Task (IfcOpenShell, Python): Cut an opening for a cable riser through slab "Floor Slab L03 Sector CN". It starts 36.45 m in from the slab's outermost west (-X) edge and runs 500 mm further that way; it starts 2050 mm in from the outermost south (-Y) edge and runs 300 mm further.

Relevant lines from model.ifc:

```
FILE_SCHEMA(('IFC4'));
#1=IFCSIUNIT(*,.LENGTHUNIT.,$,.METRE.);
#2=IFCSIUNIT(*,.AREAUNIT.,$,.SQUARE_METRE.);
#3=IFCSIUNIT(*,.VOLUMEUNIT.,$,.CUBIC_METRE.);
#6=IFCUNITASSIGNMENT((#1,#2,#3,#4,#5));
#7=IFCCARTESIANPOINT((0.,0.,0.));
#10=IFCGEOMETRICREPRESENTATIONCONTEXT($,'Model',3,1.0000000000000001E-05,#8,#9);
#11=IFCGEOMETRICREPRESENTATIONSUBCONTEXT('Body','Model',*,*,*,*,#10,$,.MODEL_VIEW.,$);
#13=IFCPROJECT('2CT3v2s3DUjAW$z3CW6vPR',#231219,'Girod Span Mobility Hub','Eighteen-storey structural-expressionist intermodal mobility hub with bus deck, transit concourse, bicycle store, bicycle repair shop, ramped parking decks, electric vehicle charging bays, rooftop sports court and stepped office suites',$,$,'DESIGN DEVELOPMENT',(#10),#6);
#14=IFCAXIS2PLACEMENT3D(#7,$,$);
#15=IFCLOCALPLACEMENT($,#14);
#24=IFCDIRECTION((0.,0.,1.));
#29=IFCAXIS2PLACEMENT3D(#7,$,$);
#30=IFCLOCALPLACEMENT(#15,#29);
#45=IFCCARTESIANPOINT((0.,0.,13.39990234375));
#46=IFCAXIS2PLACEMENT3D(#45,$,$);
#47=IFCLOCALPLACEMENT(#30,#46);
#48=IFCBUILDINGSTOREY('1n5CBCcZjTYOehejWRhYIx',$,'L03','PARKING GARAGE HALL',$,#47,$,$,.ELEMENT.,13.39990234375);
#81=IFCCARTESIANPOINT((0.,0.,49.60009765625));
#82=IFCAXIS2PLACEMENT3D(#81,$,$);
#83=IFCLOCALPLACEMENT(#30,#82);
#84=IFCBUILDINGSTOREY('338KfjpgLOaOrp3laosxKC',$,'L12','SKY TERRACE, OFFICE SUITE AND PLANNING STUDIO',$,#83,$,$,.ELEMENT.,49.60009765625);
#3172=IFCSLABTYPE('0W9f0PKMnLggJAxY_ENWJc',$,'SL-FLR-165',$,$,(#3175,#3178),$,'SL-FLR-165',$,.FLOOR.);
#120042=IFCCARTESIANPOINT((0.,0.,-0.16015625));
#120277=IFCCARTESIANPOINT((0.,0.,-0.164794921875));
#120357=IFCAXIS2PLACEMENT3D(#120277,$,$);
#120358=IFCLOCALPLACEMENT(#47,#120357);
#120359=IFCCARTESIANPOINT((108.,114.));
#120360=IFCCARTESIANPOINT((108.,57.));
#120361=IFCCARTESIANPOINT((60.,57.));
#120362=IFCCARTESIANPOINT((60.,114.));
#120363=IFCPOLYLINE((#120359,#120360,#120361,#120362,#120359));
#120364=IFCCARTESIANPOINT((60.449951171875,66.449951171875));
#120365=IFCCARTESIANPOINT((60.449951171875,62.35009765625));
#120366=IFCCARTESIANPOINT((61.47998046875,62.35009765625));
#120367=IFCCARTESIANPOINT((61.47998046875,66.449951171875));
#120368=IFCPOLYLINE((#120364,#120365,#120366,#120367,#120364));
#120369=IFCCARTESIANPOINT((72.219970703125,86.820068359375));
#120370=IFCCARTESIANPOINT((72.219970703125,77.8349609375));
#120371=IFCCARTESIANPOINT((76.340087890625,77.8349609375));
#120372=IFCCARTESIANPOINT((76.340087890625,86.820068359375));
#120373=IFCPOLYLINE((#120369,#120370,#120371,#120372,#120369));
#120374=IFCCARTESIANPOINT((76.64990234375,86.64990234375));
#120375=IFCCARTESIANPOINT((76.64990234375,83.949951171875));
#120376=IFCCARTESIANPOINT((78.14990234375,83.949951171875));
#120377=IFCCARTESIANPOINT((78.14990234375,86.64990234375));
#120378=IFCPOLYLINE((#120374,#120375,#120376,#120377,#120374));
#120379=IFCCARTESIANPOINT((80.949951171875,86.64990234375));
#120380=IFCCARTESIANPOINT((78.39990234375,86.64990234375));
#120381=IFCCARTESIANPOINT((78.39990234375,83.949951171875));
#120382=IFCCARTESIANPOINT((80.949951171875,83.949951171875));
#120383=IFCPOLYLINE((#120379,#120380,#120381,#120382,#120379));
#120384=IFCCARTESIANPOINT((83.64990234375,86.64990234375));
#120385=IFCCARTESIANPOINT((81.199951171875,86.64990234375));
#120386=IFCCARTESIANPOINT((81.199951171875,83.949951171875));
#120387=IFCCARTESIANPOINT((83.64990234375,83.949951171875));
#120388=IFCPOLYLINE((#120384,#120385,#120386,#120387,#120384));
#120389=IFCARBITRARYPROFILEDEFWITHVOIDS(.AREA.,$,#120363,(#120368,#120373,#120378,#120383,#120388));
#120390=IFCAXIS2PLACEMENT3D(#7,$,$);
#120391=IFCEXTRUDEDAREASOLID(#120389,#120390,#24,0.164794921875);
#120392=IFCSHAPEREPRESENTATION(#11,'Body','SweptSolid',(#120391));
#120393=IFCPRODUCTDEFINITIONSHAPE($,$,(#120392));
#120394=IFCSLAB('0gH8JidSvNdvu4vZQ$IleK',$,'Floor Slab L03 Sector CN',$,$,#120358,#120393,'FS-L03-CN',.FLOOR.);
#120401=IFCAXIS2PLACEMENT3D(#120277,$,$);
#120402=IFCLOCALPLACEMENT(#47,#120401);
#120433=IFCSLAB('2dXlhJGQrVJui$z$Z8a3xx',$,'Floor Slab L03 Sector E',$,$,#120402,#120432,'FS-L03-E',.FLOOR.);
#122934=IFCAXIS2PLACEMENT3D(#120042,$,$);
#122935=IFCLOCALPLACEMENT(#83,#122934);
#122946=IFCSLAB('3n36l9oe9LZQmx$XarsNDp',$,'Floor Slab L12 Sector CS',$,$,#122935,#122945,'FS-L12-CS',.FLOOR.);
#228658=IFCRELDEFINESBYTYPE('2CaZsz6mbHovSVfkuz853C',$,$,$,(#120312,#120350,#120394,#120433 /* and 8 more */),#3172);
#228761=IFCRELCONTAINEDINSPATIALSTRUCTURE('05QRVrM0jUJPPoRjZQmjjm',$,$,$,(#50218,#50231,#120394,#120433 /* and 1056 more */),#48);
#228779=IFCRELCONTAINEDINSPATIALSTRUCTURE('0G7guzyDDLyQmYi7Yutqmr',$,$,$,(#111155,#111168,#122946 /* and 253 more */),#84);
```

```python
import numpy as np
import ifcopenshell
import ifcopenshell.api.feature
import ifcopenshell.api.geometry
import ifcopenshell.api.root
import ifcopenshell.geom
import ifcopenshell.util.placement
import ifcopenshell.util.representation
import ifcopenshell.util.shape
import ifcopenshell.util.unit

model = ifcopenshell.open("model.ifc")
unit_scale = ifcopenshell.util.unit.calculate_unit_scale(model)
settings = ifcopenshell.geom.settings()


def volume(element):
    """Net volume in cubic metres, openings subtracted."""
    shape = ifcopenshell.geom.create_shape(settings, element)
    return ifcopenshell.util.shape.get_volume(shape.geometry)


slab = model.by_guid("0gH8JidSvNdvu4vZQ$IleK")
before = volume(slab)

# Extent in the slab's own axes, in metres. The edges named are its -X and -Y sides.
slab_shape = ifcopenshell.geom.create_shape(settings, slab)
vertices = ifcopenshell.util.shape.get_vertices(slab_shape.geometry)
x_min, y_min, bottom = vertices.min(axis=0)
top = vertices[:, 2].max()

opening = ifcopenshell.api.root.create_entity(model, ifc_class="IfcOpeningElement", name="Cable riser opening", predefined_type="OPENING")
context = ifcopenshell.util.representation.get_context(model, "Model", "Body", "MODEL_VIEW")
width, depth = 0.5, 0.3
outline = [(0.0, 0.0), (width, 0.0), (width, depth), (0.0, depth), (0.0, 0.0)]
# Overshoot both faces by 50 mm so the cut is clean.
shape = ifcopenshell.api.geometry.add_slab_representation(
    model, context=context, depth=top - bottom + 0.1, polyline=outline
)
ifcopenshell.api.geometry.assign_representation(model, product=opening, representation=shape)

matrix = ifcopenshell.util.placement.get_local_placement(slab.ObjectPlacement)
matrix[:, 3] = matrix @ np.append(np.array([x_min + 36.45, y_min + 2.05, bottom - 0.05]) / unit_scale, 1.0)
ifcopenshell.api.geometry.edit_object_placement(model, product=opening, matrix=matrix, is_si=False)
ifcopenshell.api.feature.add_feature(model, feature=opening, element=slab)

after = volume(slab)

print(f"slab volume {before:.3f} -> {after:.3f} m3")

model.write("model_rev.ifc")
```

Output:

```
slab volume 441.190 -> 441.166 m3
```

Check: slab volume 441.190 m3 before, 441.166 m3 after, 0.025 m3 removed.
